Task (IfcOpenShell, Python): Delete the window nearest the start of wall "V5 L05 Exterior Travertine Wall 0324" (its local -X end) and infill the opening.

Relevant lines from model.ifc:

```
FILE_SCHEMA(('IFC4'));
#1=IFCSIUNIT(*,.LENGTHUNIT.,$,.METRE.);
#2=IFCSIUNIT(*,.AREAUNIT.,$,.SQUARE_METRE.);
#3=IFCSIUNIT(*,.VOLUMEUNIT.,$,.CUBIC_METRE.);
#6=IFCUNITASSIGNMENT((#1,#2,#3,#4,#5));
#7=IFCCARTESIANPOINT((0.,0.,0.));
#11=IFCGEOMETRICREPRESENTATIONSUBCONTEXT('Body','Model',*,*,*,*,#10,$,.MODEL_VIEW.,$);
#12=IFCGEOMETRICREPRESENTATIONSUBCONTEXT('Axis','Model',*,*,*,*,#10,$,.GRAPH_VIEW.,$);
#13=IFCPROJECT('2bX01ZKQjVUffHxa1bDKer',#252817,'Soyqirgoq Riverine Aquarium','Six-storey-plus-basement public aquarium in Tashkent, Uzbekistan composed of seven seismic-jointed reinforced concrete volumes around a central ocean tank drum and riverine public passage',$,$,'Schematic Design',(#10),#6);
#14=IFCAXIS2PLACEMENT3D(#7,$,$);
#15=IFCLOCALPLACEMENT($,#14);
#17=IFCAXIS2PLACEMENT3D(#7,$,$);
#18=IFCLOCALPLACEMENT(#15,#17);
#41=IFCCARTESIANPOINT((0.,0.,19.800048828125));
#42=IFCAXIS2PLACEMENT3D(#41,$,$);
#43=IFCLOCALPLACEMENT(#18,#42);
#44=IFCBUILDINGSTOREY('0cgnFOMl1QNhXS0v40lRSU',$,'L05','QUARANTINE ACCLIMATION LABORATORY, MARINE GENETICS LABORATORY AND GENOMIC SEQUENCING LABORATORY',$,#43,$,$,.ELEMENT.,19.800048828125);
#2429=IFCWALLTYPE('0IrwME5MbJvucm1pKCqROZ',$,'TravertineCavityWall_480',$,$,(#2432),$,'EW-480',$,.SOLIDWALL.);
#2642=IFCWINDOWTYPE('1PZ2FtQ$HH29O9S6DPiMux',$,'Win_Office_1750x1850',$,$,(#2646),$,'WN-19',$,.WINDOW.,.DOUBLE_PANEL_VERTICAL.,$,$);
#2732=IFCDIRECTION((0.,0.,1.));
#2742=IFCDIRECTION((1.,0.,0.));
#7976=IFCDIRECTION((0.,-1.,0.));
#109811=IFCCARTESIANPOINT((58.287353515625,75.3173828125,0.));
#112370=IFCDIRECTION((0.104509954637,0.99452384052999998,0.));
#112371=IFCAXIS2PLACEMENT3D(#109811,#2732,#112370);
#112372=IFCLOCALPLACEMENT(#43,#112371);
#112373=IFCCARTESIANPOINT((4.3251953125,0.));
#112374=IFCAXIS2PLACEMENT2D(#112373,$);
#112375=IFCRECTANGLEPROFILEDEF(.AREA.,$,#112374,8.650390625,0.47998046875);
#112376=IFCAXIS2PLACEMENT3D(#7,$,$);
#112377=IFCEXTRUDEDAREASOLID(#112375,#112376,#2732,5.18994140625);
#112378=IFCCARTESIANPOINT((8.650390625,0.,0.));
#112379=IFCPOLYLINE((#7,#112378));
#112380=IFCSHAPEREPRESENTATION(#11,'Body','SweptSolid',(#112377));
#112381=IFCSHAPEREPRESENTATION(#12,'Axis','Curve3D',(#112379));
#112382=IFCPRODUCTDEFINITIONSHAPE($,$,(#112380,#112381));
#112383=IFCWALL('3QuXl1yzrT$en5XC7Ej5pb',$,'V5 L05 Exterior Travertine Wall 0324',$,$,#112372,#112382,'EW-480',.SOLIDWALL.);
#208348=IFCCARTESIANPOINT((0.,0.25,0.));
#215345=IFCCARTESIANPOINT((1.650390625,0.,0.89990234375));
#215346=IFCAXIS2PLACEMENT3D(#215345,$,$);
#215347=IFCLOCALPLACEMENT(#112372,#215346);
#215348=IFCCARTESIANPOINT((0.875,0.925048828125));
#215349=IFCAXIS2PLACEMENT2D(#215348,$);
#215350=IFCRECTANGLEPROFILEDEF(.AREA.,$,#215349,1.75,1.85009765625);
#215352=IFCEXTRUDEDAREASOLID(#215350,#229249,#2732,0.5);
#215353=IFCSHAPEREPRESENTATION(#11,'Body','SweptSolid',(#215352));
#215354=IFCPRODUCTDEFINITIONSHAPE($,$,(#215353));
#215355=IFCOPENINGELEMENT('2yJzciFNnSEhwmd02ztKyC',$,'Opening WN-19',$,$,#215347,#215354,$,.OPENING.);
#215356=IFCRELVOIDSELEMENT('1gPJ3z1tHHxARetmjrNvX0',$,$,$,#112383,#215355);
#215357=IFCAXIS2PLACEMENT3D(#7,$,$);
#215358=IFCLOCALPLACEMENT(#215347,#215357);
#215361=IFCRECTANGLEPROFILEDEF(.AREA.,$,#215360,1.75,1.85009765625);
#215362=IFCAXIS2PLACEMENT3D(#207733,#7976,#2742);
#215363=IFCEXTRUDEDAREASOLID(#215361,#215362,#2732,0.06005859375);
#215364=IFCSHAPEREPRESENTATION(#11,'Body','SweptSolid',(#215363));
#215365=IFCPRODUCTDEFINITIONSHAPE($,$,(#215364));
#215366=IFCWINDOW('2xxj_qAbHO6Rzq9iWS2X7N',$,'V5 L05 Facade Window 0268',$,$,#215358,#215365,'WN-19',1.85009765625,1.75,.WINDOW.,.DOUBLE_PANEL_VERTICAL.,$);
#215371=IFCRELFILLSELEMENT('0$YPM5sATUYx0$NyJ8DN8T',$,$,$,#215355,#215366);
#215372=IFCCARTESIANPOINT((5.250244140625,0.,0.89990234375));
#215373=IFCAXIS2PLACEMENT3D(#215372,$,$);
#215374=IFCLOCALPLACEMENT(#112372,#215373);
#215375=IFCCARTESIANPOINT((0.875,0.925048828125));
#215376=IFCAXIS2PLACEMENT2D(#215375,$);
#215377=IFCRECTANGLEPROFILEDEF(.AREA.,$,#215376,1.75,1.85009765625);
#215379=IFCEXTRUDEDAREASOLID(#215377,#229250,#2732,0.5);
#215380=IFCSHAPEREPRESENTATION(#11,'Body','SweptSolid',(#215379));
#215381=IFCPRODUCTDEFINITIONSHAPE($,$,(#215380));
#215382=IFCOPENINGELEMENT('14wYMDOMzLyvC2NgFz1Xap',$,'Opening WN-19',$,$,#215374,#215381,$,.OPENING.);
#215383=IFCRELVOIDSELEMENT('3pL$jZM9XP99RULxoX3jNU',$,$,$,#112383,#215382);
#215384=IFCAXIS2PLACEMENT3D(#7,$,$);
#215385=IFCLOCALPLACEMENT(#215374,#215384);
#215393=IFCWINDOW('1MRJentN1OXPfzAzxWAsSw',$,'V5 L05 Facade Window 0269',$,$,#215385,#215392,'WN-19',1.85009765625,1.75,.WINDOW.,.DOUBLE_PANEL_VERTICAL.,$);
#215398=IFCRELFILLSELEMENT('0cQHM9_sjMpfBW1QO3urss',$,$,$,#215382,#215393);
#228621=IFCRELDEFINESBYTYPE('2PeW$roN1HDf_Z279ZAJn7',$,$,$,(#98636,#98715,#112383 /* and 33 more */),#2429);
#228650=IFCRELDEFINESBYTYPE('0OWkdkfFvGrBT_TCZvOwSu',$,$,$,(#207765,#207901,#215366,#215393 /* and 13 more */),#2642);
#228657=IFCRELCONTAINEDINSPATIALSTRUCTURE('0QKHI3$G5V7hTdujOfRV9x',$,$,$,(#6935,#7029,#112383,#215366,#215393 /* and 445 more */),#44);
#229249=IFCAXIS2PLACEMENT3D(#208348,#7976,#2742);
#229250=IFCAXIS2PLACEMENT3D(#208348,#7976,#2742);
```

```python
import ifcopenshell
import ifcopenshell.api.feature
import ifcopenshell.api.root
import ifcopenshell.geom
import ifcopenshell.util.shape

model = ifcopenshell.open("model.ifc")
settings = ifcopenshell.geom.settings()


def volume(element):
    """Net volume in cubic metres, openings subtracted."""
    shape = ifcopenshell.geom.create_shape(settings, element)
    return ifcopenshell.util.shape.get_volume(shape.geometry)


window = model.by_id(215366)
opening = window.FillsVoids[0].RelatingOpeningElement
wall = opening.VoidsElements[0].RelatingBuildingElement
before = volume(wall)

ifcopenshell.api.root.remove_product(model, product=window)
ifcopenshell.api.feature.remove_feature(model, feature=opening)

after = volume(wall)

print(f"wall volume {before:.3f} -> {after:.3f} m3")

model.write("model_v2.ifc")
```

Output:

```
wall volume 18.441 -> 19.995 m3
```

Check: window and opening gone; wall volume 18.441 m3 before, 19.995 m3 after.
